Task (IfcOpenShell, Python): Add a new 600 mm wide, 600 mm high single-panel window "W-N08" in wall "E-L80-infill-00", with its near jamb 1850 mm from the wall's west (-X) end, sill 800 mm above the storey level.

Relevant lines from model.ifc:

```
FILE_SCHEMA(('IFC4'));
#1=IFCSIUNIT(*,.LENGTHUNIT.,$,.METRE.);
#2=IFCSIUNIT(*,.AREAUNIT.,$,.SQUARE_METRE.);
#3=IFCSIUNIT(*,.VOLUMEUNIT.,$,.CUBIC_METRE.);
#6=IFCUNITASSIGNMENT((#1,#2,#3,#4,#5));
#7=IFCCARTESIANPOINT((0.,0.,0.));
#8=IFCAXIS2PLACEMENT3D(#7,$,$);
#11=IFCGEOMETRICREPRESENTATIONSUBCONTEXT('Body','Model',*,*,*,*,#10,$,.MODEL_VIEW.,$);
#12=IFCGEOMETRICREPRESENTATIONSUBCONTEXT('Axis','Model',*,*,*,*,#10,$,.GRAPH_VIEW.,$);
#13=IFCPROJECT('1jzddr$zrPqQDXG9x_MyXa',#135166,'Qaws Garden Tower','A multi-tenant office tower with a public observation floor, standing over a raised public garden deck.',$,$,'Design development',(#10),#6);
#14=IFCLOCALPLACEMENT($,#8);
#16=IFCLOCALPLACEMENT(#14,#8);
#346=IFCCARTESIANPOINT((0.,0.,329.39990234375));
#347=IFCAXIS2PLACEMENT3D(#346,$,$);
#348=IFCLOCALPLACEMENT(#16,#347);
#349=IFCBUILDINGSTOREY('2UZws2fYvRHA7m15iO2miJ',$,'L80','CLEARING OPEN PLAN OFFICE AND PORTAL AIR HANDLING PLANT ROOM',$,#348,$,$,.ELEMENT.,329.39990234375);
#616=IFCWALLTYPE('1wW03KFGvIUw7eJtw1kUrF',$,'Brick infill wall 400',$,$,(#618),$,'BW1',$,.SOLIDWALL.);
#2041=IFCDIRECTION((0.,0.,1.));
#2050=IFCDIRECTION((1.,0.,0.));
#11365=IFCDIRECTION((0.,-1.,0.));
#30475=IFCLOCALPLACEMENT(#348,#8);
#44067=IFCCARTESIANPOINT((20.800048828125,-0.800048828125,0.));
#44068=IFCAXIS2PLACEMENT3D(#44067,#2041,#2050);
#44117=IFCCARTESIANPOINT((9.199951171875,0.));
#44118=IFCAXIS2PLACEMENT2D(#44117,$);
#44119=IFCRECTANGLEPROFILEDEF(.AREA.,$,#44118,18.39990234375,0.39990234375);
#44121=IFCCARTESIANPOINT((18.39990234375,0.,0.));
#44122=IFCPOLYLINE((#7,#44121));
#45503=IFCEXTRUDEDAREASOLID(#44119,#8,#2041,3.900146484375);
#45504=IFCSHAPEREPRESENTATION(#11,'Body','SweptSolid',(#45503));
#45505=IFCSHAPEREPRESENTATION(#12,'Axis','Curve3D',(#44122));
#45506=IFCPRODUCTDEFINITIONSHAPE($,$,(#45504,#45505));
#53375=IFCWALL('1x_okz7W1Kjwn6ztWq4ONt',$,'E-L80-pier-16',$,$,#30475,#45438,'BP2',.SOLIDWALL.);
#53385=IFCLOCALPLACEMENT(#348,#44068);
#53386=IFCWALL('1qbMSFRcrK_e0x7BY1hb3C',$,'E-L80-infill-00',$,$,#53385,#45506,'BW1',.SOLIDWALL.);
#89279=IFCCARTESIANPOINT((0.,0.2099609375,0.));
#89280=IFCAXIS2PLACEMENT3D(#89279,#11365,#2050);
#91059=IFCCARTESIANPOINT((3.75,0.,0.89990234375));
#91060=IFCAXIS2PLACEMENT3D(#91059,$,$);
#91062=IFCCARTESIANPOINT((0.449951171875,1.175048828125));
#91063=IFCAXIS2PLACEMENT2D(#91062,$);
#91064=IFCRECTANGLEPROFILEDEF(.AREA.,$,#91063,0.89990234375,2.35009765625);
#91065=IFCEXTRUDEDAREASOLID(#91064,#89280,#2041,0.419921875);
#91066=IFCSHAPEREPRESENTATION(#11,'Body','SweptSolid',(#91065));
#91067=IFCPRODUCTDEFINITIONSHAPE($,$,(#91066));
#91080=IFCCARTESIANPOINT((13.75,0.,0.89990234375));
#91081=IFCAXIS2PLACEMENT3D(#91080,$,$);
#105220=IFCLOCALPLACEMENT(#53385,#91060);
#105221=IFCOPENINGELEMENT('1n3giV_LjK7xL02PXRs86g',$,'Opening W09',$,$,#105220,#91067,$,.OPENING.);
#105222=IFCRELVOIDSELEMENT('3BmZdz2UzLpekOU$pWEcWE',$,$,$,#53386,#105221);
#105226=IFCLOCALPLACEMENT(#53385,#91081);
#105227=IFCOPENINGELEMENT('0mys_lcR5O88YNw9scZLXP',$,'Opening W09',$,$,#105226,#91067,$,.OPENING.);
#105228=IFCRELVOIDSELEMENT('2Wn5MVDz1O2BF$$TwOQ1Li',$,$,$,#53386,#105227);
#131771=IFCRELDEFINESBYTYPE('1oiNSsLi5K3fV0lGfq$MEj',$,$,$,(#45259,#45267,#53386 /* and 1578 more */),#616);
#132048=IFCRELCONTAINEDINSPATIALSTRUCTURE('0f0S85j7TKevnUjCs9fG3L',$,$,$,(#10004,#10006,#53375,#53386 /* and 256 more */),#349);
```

```python
import numpy as np
import ifcopenshell
import ifcopenshell.api.feature
import ifcopenshell.api.geometry
import ifcopenshell.api.root
import ifcopenshell.api.spatial
import ifcopenshell.geom
import ifcopenshell.util.element
import ifcopenshell.util.placement
import ifcopenshell.util.representation
import ifcopenshell.util.shape
import ifcopenshell.util.unit

model = ifcopenshell.open("model.ifc")
unit_scale = ifcopenshell.util.unit.calculate_unit_scale(model)
settings = ifcopenshell.geom.settings()


def volume(element):
    """Net volume in cubic metres, openings subtracted."""
    shape = ifcopenshell.geom.create_shape(settings, element)
    return ifcopenshell.util.shape.get_volume(shape.geometry)


wall = model.by_guid("1qbMSFRcrK_e0x7BY1hb3C")
storey = ifcopenshell.util.element.get_container(wall, ifc_class="IfcBuildingStorey")
context = ifcopenshell.util.representation.get_context(model, "Model", "Body", "MODEL_VIEW")
before = volume(wall)

width, height, from_end, sill = 0.6, 0.6, 1.85, 0.8  # metres

# The wall runs along its own X axis, and the end named is its -X end.
wall_shape = ifcopenshell.geom.create_shape(settings, wall)
x, y, z = ifcopenshell.util.shape.get_vertices(wall_shape.geometry).T
start = x.min() + from_end
face, thickness = float(y.min()), float(y.max() - y.min())
wall_matrix = ifcopenshell.util.placement.get_local_placement(wall.ObjectPlacement)
level = ifcopenshell.util.placement.get_local_placement(storey.ObjectPlacement)[2, 3]


def in_wall(x, y):
    """Placement at x, y metres in the wall's axes, at sill height."""
    matrix = wall_matrix.copy()
    matrix[:, 3] = wall_matrix @ np.array([x / unit_scale, y / unit_scale, 0.0, 1.0])
    matrix[2, 3] = level + sill / unit_scale
    return matrix


# Opening: a box that overshoots both wall faces by 50 mm.
opening = ifcopenshell.api.root.create_entity(model, ifc_class="IfcOpeningElement", predefined_type="OPENING")
box = ifcopenshell.api.geometry.add_wall_representation(
    model, context=context, length=width, height=height, thickness=thickness + 0.1
)
ifcopenshell.api.geometry.assign_representation(model, product=opening, representation=box)
ifcopenshell.api.geometry.edit_object_placement(model, product=opening, matrix=in_wall(start, face - 0.05), is_si=False)
ifcopenshell.api.feature.add_feature(model, feature=opening, element=wall)

window = ifcopenshell.api.root.create_entity(model, ifc_class="IfcWindow", name="W-N08", predefined_type="WINDOW")
window.OverallWidth, window.OverallHeight = width / unit_scale, height / unit_scale
window.PartitioningType = "SINGLE_PANEL"
body = ifcopenshell.api.geometry.add_window_representation(
    model,
    context=context,
    overall_width=window.OverallWidth,
    overall_height=window.OverallHeight,
    partition_type="SINGLE_PANEL",
)
ifcopenshell.api.geometry.assign_representation(model, product=window, representation=body)
ifcopenshell.api.spatial.assign_container(model, products=[window], relating_structure=storey)
ifcopenshell.api.feature.add_filling(model, opening=opening, element=window)

# Centre the window in the wall's thickness.
ifcopenshell.api.geometry.edit_object_placement(model, product=window, matrix=in_wall(start, face), is_si=False)
window_shape = ifcopenshell.geom.create_shape(settings, window)
depth = ifcopenshell.util.shape.get_vertices(window_shape.geometry)[:, 1]
offset = face + thickness / 2 - (depth.min() + depth.max()) / 2
ifcopenshell.api.geometry.edit_object_placement(model, product=window, matrix=in_wall(start, offset), is_si=False)

after = volume(wall)

print(f"wall volume {before:.3f} -> {after:.3f} m3")

model.write("model_v2.ifc")
```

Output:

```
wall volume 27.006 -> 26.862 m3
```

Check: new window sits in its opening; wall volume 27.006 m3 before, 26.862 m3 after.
